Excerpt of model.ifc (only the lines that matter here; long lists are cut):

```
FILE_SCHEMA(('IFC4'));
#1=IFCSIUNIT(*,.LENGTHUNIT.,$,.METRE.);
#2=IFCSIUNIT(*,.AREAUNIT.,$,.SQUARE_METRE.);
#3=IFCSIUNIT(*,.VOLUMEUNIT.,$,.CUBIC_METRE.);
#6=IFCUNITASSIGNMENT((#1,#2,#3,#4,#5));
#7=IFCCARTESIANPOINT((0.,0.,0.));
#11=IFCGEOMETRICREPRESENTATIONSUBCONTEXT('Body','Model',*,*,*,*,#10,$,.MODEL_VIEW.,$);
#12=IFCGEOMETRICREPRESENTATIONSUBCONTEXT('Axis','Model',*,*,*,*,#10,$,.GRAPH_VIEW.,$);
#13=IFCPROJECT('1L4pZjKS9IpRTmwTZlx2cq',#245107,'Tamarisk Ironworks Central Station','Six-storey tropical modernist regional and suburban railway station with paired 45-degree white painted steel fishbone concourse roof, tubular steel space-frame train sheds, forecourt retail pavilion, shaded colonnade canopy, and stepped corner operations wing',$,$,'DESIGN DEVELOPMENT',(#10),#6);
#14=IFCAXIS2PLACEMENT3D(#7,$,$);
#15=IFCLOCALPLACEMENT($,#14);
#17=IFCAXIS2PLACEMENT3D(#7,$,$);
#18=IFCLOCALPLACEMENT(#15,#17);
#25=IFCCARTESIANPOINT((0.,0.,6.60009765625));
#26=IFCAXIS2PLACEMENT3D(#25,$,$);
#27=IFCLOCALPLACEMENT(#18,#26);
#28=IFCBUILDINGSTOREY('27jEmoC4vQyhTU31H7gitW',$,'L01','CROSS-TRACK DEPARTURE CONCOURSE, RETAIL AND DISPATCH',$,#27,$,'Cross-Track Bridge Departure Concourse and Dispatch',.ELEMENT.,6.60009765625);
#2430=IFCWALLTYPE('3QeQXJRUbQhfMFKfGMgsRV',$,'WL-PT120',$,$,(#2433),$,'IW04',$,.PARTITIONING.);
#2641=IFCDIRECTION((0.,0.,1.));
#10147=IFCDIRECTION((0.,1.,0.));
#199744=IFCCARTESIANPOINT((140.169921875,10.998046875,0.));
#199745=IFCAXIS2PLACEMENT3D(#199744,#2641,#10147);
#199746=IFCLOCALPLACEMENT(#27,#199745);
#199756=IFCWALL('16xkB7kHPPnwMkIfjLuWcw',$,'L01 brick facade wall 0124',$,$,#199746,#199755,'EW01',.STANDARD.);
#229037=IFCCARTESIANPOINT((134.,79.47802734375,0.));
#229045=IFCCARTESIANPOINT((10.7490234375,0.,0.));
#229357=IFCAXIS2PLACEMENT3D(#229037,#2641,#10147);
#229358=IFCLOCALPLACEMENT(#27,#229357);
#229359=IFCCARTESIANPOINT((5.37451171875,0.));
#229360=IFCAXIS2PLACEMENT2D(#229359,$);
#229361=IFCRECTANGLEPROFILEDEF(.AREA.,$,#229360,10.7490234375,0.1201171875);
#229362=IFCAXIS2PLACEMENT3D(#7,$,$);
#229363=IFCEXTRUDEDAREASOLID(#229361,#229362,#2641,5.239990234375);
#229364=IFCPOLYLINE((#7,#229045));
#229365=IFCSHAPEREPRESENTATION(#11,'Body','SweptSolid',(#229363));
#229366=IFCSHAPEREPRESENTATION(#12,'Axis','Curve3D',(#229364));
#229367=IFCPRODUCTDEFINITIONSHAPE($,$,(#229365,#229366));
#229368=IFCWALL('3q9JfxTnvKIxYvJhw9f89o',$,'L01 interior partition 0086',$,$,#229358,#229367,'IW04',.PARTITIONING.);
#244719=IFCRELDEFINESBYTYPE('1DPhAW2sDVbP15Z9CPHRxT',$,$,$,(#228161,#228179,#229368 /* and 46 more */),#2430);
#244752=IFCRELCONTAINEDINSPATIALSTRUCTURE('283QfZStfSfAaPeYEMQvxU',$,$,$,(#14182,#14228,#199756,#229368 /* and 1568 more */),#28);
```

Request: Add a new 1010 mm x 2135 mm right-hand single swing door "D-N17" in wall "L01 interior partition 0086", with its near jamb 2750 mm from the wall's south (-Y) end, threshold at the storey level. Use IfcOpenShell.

```python
import numpy as np
import ifcopenshell
import ifcopenshell.api.feature
import ifcopenshell.api.geometry
import ifcopenshell.api.root
import ifcopenshell.api.spatial
import ifcopenshell.geom
import ifcopenshell.util.element
import ifcopenshell.util.placement
import ifcopenshell.util.representation
import ifcopenshell.util.shape
import ifcopenshell.util.unit

model = ifcopenshell.open("model.ifc")
unit_scale = ifcopenshell.util.unit.calculate_unit_scale(model)
settings = ifcopenshell.geom.settings()


def volume(element):
    """Net volume in cubic metres, openings subtracted."""
    shape = ifcopenshell.geom.create_shape(settings, element)
    return ifcopenshell.util.shape.get_volume(shape.geometry)


wall = model.by_guid("3q9JfxTnvKIxYvJhw9f89o")
storey = ifcopenshell.util.element.get_container(wall, ifc_class="IfcBuildingStorey")
context = ifcopenshell.util.representation.get_context(model, "Model", "Body", "MODEL_VIEW")
before = volume(wall)

width, height, from_end, sill = 1.01, 2.135, 2.75, 0.0  # metres

# The wall runs along its own X axis, and the end named is its -X end.
wall_shape = ifcopenshell.geom.create_shape(settings, wall)
x, y, z = ifcopenshell.util.shape.get_vertices(wall_shape.geometry).T
start = x.min() + from_end
face, thickness = float(y.min()), float(y.max() - y.min())
wall_matrix = ifcopenshell.util.placement.get_local_placement(wall.ObjectPlacement)
level = ifcopenshell.util.placement.get_local_placement(storey.ObjectPlacement)[2, 3]


def in_wall(x, y):
    """Placement at x, y metres in the wall's axes, at sill height."""
    matrix = wall_matrix.copy()
    matrix[:, 3] = wall_matrix @ np.array([x / unit_scale, y / unit_scale, 0.0, 1.0])
    matrix[2, 3] = level + sill / unit_scale
    return matrix


# Opening: a box that overshoots both wall faces by 50 mm.
opening = ifcopenshell.api.root.create_entity(model, ifc_class="IfcOpeningElement", predefined_type="OPENING")
box = ifcopenshell.api.geometry.add_wall_representation(
    model, context=context, length=width, height=height, thickness=thickness + 0.1
)
ifcopenshell.api.geometry.assign_representation(model, product=opening, representation=box)
ifcopenshell.api.geometry.edit_object_placement(model, product=opening, matrix=in_wall(start, face - 0.05), is_si=False)
ifcopenshell.api.feature.add_feature(model, feature=opening, element=wall)

door = ifcopenshell.api.root.create_entity(model, ifc_class="IfcDoor", name="D-N17", predefined_type="DOOR")
door.OverallWidth, door.OverallHeight = width / unit_scale, height / unit_scale
door.OperationType = "SINGLE_SWING_RIGHT"
body = ifcopenshell.api.geometry.add_door_representation(
    model,
    context=context,
    overall_width=door.OverallWidth,
    overall_height=door.OverallHeight,
    operation_type="SINGLE_SWING_RIGHT",
    lining_properties={"LiningDepth": thickness / unit_scale, "ThresholdDepth": thickness / unit_scale},
)
ifcopenshell.api.geometry.assign_representation(model, product=door, representation=body)
ifcopenshell.api.spatial.assign_container(model, products=[door], relating_structure=storey)
ifcopenshell.api.feature.add_filling(model, opening=opening, element=door)

# The lining spans the wall, so the door starts at the wall face.
ifcopenshell.api.geometry.edit_object_placement(model, product=door, matrix=in_wall(start, face), is_si=False)

after = volume(wall)

print(f"wall volume {before:.3f} -> {after:.3f} m3")

model.write("model_rev.ifc")
```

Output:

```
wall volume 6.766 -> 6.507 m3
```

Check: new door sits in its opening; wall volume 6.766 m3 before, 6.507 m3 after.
